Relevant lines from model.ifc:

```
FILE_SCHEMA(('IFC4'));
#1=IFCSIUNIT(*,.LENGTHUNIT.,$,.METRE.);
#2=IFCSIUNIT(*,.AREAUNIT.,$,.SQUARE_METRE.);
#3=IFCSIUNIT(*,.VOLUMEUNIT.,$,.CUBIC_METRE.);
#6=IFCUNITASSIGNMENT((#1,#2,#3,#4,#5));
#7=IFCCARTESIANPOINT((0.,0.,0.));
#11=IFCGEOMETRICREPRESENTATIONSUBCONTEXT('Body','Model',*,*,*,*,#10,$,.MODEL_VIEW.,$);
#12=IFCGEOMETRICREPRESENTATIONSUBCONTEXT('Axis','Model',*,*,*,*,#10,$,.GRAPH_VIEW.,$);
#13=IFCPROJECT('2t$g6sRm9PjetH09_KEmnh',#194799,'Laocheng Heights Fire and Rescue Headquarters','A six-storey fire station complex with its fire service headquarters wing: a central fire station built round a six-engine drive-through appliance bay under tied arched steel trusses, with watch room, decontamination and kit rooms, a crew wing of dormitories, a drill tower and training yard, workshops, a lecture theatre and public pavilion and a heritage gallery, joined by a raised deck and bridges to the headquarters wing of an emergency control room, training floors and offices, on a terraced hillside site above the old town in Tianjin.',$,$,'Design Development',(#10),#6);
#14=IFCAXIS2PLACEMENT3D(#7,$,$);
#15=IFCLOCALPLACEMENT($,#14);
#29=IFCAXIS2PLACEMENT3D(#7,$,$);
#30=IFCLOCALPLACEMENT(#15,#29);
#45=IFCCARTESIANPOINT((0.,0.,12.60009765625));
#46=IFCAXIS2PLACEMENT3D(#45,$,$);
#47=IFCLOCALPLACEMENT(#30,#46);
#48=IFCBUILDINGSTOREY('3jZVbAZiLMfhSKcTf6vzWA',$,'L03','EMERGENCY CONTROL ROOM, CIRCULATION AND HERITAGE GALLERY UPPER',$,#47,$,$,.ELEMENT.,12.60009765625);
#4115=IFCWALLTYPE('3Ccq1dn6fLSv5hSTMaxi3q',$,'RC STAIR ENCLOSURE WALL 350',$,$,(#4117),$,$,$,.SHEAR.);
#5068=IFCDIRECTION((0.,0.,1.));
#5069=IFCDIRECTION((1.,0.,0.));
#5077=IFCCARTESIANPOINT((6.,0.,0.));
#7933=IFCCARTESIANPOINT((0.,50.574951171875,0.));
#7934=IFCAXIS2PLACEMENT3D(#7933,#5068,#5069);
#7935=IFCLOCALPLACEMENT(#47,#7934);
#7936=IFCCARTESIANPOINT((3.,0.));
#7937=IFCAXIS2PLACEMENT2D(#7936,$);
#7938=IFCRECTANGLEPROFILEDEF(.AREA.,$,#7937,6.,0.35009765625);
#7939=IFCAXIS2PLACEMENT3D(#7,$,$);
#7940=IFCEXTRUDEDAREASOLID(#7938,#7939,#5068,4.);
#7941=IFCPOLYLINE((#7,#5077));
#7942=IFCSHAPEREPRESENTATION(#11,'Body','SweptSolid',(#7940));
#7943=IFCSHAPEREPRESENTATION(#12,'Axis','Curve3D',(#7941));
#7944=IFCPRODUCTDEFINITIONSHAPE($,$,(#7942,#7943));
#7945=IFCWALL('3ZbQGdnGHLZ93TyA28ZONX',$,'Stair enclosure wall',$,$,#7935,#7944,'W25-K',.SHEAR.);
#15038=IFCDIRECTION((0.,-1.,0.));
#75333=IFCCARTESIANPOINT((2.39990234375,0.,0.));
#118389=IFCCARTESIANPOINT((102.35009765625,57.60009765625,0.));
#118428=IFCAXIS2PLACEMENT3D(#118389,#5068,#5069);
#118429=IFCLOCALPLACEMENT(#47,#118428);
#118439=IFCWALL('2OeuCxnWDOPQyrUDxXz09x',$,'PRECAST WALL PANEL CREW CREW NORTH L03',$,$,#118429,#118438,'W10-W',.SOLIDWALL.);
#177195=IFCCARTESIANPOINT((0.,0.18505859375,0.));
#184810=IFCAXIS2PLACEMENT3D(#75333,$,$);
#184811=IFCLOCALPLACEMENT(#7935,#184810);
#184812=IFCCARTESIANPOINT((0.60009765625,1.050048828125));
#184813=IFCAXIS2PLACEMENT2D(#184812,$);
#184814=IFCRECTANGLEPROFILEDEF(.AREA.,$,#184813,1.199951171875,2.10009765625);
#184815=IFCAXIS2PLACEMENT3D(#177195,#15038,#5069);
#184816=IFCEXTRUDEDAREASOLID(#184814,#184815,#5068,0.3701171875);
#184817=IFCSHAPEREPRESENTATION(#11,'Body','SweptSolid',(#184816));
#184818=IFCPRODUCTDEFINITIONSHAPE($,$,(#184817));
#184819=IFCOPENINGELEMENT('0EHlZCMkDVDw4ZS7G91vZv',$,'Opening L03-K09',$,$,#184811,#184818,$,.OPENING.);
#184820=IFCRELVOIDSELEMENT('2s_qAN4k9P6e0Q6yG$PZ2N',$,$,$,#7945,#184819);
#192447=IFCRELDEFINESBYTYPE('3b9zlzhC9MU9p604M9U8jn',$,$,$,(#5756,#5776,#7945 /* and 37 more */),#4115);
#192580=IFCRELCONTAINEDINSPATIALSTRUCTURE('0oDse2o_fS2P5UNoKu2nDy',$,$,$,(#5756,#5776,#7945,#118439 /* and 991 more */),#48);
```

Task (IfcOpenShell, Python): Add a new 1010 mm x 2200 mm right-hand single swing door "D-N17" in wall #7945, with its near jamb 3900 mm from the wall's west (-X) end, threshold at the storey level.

```python
import numpy as np
import ifcopenshell
import ifcopenshell.api.feature
import ifcopenshell.api.geometry
import ifcopenshell.api.root
import ifcopenshell.api.spatial
import ifcopenshell.geom
import ifcopenshell.util.element
import ifcopenshell.util.placement
import ifcopenshell.util.representation
import ifcopenshell.util.shape
import ifcopenshell.util.unit

model = ifcopenshell.open("model.ifc")
unit_scale = ifcopenshell.util.unit.calculate_unit_scale(model)
settings = ifcopenshell.geom.settings()


def volume(element):
    """Net volume in cubic metres, openings subtracted."""
    shape = ifcopenshell.geom.create_shape(settings, element)
    return ifcopenshell.util.shape.get_volume(shape.geometry)


wall = model.by_id(7945)
storey = ifcopenshell.util.element.get_container(wall, ifc_class="IfcBuildingStorey")
context = ifcopenshell.util.representation.get_context(model, "Model", "Body", "MODEL_VIEW")
before = volume(wall)

width, height, from_end, sill = 1.01, 2.2, 3.9, 0.0  # metres

# The wall runs along its own X axis, and the end named is its -X end.
wall_shape = ifcopenshell.geom.create_shape(settings, wall)
x, y, z = ifcopenshell.util.shape.get_vertices(wall_shape.geometry).T
start = x.min() + from_end
face, thickness = float(y.min()), float(y.max() - y.min())
wall_matrix = ifcopenshell.util.placement.get_local_placement(wall.ObjectPlacement)
level = ifcopenshell.util.placement.get_local_placement(storey.ObjectPlacement)[2, 3]


def in_wall(x, y):
    """Placement at x, y metres in the wall's axes, at sill height."""
    matrix = wall_matrix.copy()
    matrix[:, 3] = wall_matrix @ np.array([x / unit_scale, y / unit_scale, 0.0, 1.0])
    matrix[2, 3] = level + sill / unit_scale
    return matrix


# Opening: a box that overshoots both wall faces by 50 mm.
opening = ifcopenshell.api.root.create_entity(model, ifc_class="IfcOpeningElement", predefined_type="OPENING")
box = ifcopenshell.api.geometry.add_wall_representation(
    model, context=context, length=width, height=height, thickness=thickness + 0.1
)
ifcopenshell.api.geometry.assign_representation(model, product=opening, representation=box)
ifcopenshell.api.geometry.edit_object_placement(model, product=opening, matrix=in_wall(start, face - 0.05), is_si=False)
ifcopenshell.api.feature.add_feature(model, feature=opening, element=wall)

door = ifcopenshell.api.root.create_entity(model, ifc_class="IfcDoor", name="D-N17", predefined_type="DOOR")
door.OverallWidth, door.OverallHeight = width / unit_scale, height / unit_scale
door.OperationType = "SINGLE_SWING_RIGHT"
body = ifcopenshell.api.geometry.add_door_representation(
    model,
    context=context,
    overall_width=door.OverallWidth,
    overall_height=door.OverallHeight,
    operation_type="SINGLE_SWING_RIGHT",
    lining_properties={"LiningDepth": thickness / unit_scale, "ThresholdDepth": thickness / unit_scale},
)
ifcopenshell.api.geometry.assign_representation(model, product=door, representation=body)
ifcopenshell.api.spatial.assign_container(model, products=[door], relating_structure=storey)
ifcopenshell.api.feature.add_filling(model, opening=opening, element=door)

# The lining spans the wall, so the door starts at the wall face.
ifcopenshell.api.geometry.edit_object_placement(model, product=door, matrix=in_wall(start, face), is_si=False)

after = volume(wall)

print(f"wall volume {before:.3f} -> {after:.3f} m3")

model.write("model_rev.ifc")
```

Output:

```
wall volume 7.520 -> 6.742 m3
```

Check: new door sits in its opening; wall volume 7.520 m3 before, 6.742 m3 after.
